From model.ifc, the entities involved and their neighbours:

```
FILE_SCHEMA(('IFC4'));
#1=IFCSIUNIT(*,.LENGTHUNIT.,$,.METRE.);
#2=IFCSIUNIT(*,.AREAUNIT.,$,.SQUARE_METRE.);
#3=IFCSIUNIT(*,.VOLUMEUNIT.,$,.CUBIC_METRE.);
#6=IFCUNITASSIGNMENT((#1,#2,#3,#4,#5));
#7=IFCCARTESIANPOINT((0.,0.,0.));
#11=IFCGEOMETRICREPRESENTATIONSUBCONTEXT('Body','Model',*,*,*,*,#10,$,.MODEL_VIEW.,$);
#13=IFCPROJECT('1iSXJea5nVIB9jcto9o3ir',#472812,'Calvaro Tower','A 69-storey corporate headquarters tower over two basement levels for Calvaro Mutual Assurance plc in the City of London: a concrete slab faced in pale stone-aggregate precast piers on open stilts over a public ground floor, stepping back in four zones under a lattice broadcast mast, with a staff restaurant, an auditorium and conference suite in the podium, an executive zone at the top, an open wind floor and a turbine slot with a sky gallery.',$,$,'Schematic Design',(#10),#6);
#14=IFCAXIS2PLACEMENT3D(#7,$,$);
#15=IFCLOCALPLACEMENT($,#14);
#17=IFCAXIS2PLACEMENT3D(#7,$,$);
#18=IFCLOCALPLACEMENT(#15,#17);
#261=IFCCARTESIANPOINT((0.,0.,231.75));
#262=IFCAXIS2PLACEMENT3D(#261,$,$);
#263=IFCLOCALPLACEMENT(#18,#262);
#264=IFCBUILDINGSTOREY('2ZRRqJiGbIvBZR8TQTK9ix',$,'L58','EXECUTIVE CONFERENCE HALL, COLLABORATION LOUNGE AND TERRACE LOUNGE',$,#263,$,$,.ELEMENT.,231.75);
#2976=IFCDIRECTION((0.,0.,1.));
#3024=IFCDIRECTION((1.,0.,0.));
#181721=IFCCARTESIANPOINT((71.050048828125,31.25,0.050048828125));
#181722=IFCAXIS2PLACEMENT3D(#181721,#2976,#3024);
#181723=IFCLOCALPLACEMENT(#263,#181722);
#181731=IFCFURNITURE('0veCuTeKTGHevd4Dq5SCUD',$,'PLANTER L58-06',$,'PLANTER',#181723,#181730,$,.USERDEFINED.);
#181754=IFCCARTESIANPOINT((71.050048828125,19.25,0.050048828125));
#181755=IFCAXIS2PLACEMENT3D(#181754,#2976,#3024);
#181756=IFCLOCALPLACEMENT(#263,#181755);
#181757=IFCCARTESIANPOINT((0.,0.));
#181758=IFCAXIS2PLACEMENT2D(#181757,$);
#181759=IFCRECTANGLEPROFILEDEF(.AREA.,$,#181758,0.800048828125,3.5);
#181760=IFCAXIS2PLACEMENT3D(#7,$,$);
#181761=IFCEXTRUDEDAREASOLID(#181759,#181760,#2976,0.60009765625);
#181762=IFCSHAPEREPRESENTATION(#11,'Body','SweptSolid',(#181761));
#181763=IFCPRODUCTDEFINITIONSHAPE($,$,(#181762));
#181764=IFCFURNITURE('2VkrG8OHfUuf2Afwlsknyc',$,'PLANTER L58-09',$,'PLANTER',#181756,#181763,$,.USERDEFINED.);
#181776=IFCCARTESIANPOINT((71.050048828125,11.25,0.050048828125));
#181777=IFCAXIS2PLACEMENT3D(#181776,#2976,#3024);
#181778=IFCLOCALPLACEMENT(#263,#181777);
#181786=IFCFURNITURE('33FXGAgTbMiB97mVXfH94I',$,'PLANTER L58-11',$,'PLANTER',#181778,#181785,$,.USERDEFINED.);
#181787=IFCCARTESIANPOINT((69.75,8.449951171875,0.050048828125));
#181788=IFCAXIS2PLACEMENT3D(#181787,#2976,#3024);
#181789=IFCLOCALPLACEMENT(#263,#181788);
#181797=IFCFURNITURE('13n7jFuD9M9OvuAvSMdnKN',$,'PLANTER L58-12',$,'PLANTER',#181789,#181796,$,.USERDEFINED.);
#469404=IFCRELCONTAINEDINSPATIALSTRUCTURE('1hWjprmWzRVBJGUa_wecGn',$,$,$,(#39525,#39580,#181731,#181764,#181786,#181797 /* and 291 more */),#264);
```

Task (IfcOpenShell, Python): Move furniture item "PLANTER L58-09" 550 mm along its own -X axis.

```python
import ifcopenshell
import ifcopenshell.api.geometry
import ifcopenshell.util.placement
import ifcopenshell.util.unit

model = ifcopenshell.open("model.ifc")
unit_scale = ifcopenshell.util.unit.calculate_unit_scale(model)

item = model.by_guid("2VkrG8OHfUuf2Afwlsknyc")
matrix = ifcopenshell.util.placement.get_local_placement(item.ObjectPlacement)
matrix[:3, 3] -= matrix[:3, 0] * 0.55 / unit_scale
ifcopenshell.api.geometry.edit_object_placement(model, product=item, matrix=matrix, is_si=False)

print(ifcopenshell.util.placement.get_local_placement(item.ObjectPlacement).round(3) + 0.0)

model.write("model-out.ifc")
```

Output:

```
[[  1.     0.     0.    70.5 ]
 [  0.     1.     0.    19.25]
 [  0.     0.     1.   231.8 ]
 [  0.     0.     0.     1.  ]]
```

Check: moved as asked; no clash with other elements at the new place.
